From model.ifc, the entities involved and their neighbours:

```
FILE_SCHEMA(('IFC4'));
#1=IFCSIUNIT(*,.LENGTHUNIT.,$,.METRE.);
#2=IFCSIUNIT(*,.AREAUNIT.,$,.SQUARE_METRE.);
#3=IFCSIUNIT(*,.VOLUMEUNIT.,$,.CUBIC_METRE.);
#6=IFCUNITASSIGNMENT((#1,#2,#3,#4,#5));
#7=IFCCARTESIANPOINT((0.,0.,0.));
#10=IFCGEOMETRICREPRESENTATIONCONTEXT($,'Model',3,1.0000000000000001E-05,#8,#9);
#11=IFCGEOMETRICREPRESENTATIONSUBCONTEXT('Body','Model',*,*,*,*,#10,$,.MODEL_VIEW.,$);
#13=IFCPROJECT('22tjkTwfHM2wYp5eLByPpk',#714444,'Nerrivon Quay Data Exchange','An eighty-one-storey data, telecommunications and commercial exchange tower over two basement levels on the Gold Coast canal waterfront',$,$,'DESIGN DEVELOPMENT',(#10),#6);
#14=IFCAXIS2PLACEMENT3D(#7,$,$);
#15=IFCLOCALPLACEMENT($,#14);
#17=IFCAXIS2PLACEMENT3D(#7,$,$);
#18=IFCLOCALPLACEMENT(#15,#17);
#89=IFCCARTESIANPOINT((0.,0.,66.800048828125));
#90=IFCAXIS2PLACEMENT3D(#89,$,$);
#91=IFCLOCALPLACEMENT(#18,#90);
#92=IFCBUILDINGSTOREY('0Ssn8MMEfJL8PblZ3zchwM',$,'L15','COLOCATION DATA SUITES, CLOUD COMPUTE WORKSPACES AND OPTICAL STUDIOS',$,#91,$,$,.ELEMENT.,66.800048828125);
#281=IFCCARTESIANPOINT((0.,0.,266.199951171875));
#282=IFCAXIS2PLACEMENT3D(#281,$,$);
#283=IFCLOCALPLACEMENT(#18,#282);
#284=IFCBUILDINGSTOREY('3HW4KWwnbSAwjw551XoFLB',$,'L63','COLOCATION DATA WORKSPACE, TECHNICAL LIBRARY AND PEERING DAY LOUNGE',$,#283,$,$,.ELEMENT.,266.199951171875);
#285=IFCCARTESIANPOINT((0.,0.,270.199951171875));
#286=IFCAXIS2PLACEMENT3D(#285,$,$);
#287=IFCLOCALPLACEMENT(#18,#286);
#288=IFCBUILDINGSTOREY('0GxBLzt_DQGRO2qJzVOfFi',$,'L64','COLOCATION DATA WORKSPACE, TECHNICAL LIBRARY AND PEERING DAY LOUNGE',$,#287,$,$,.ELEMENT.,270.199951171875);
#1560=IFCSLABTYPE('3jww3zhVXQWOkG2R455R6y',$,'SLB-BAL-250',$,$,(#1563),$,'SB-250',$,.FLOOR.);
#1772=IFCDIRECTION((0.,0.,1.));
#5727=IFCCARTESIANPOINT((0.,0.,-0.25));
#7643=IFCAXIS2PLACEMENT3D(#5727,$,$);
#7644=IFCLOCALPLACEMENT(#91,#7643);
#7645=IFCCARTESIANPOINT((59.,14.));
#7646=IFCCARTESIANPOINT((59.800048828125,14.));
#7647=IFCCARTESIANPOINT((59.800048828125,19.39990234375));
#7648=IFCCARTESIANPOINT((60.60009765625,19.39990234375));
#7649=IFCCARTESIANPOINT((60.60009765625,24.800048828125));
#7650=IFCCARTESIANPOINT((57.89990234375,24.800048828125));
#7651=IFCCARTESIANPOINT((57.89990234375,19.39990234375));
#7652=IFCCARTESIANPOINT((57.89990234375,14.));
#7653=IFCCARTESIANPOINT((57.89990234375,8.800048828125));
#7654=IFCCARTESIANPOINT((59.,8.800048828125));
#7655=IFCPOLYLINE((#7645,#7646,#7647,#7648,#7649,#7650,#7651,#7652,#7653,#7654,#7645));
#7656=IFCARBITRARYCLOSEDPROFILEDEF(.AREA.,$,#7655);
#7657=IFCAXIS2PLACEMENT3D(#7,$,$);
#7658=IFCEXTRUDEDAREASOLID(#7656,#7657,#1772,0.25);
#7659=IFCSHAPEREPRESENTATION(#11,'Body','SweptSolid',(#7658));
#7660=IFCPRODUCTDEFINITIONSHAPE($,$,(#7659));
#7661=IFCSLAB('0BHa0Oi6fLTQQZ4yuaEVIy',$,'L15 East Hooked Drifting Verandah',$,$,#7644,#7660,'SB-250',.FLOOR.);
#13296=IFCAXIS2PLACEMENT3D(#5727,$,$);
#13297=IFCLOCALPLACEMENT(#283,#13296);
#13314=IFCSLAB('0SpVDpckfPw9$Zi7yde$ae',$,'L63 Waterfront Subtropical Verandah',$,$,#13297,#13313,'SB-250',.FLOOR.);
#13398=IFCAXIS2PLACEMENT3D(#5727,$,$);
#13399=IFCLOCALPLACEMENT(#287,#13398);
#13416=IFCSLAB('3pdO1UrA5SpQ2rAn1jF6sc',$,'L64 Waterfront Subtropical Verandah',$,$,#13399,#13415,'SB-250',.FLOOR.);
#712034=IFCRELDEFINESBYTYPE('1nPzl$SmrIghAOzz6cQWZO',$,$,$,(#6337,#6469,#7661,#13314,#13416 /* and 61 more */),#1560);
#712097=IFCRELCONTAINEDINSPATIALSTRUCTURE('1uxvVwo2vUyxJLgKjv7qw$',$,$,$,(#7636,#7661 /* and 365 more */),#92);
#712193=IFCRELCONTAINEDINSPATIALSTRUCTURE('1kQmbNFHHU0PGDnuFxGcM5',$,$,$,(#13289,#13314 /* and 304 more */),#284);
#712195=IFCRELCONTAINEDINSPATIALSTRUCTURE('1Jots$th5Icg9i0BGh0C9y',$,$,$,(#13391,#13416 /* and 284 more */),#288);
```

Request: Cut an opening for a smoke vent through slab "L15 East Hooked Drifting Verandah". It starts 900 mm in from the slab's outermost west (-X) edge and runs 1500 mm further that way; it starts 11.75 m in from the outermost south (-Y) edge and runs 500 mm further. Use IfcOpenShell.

```python
import numpy as np
import ifcopenshell
import ifcopenshell.api.feature
import ifcopenshell.api.geometry
import ifcopenshell.api.root
import ifcopenshell.geom
import ifcopenshell.util.placement
import ifcopenshell.util.representation
import ifcopenshell.util.shape
import ifcopenshell.util.unit

model = ifcopenshell.open("model.ifc")
unit_scale = ifcopenshell.util.unit.calculate_unit_scale(model)
settings = ifcopenshell.geom.settings()


def volume(element):
    """Net volume in cubic metres, openings subtracted."""
    shape = ifcopenshell.geom.create_shape(settings, element)
    return ifcopenshell.util.shape.get_volume(shape.geometry)


slab = model.by_id(7661)
before = volume(slab)

# Extent in the slab's own axes, in metres. The edges named are its -X and -Y sides.
slab_shape = ifcopenshell.geom.create_shape(settings, slab)
vertices = ifcopenshell.util.shape.get_vertices(slab_shape.geometry)
x_min, y_min, bottom = vertices.min(axis=0)
top = vertices[:, 2].max()

opening = ifcopenshell.api.root.create_entity(model, ifc_class="IfcOpeningElement", name="Smoke vent opening", predefined_type="OPENING")
context = ifcopenshell.util.representation.get_context(model, "Model", "Body", "MODEL_VIEW")
width, depth = 1.5, 0.5
outline = [(0.0, 0.0), (width, 0.0), (width, depth), (0.0, depth), (0.0, 0.0)]
# Overshoot both faces by 50 mm so the cut is clean.
shape = ifcopenshell.api.geometry.add_slab_representation(
    model, context=context, depth=top - bottom + 0.1, polyline=outline
)
ifcopenshell.api.geometry.assign_representation(model, product=opening, representation=shape)

matrix = ifcopenshell.util.placement.get_local_placement(slab.ObjectPlacement)
matrix[:, 3] = matrix @ np.append(np.array([x_min + 0.9, y_min + 11.75, bottom - 0.05]) / unit_scale, 1.0)
ifcopenshell.api.geometry.edit_object_placement(model, product=opening, matrix=matrix, is_si=False)
ifcopenshell.api.feature.add_feature(model, feature=opening, element=slab)

after = volume(slab)

print(f"slab volume {before:.3f} -> {after:.3f} m3")

model.write("model_rev.ifc")
```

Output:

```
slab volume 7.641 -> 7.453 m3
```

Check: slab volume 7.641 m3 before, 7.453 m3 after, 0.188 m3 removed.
